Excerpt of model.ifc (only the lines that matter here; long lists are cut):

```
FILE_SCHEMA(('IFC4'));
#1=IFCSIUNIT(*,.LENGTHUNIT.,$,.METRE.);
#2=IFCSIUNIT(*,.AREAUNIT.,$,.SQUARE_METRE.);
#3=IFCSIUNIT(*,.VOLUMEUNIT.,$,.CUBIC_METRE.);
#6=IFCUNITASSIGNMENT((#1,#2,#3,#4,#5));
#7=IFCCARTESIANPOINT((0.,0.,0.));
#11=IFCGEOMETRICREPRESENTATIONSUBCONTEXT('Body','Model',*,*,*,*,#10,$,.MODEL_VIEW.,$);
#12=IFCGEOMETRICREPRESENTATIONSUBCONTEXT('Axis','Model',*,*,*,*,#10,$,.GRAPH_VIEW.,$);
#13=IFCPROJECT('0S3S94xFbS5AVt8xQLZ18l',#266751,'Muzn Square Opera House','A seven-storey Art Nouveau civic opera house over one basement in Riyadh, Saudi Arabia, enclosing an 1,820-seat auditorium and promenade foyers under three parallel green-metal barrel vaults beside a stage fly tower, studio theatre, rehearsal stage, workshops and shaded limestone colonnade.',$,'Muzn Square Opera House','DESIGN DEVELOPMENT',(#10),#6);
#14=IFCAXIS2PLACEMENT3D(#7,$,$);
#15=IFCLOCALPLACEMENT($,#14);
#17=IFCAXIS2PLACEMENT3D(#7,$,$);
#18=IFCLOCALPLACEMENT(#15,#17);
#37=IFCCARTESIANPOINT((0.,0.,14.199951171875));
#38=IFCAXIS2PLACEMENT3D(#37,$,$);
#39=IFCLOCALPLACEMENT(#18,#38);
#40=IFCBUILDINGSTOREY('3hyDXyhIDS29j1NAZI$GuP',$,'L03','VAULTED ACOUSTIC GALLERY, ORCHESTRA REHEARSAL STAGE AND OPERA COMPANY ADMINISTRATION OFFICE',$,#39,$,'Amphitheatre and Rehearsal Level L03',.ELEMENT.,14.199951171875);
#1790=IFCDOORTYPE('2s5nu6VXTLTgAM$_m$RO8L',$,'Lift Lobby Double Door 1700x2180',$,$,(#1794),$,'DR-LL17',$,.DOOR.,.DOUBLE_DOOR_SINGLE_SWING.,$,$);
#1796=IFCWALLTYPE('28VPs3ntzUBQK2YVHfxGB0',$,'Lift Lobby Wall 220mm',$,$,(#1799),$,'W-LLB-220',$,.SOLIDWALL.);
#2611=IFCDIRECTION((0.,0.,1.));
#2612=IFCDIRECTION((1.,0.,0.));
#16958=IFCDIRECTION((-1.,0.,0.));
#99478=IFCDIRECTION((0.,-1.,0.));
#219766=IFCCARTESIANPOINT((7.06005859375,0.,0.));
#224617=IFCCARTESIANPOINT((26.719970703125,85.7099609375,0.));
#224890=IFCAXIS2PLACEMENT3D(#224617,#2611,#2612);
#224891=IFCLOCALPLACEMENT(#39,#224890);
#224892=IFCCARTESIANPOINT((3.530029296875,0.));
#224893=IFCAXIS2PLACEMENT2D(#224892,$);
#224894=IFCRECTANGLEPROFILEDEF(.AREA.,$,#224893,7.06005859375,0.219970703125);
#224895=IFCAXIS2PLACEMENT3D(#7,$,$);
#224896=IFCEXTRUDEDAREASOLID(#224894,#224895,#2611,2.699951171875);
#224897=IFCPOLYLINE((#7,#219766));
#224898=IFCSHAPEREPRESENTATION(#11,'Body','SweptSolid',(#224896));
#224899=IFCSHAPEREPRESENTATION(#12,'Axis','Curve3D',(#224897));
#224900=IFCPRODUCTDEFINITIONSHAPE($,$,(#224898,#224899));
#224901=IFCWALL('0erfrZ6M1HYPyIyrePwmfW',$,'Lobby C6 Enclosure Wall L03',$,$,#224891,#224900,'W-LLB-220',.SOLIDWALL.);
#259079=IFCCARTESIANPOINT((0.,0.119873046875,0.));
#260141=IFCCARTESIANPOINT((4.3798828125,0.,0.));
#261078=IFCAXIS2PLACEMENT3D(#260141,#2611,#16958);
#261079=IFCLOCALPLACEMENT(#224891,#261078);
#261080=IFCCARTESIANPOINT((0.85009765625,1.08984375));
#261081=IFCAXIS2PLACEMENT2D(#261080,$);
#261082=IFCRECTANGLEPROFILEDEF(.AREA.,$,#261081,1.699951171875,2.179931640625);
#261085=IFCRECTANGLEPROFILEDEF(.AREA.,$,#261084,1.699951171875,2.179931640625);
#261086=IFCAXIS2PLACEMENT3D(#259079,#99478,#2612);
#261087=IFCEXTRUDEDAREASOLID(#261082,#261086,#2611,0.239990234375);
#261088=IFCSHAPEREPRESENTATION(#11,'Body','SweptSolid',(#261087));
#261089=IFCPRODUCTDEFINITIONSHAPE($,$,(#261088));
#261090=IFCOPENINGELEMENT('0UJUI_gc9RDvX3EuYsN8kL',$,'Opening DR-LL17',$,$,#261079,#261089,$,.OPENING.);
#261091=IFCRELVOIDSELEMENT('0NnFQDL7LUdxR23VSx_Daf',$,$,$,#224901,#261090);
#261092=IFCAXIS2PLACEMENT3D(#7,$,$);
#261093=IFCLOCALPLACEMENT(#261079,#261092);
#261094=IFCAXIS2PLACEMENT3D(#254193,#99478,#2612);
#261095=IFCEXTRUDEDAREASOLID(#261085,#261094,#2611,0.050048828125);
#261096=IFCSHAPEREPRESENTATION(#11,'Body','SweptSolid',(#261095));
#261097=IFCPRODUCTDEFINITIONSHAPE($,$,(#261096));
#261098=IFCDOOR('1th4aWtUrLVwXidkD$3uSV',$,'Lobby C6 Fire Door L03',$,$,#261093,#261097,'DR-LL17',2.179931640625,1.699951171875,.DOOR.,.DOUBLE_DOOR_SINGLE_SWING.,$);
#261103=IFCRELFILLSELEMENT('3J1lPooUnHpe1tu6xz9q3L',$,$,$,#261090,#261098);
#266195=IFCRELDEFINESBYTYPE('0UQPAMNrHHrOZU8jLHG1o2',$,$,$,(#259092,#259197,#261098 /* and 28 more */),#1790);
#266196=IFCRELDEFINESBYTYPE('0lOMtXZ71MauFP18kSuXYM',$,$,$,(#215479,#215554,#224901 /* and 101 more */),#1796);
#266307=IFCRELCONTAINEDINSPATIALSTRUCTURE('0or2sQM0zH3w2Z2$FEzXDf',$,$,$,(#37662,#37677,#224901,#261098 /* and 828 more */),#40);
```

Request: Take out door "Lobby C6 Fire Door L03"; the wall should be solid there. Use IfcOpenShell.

```python
import ifcopenshell
import ifcopenshell.api.feature
import ifcopenshell.api.root
import ifcopenshell.geom
import ifcopenshell.util.shape

model = ifcopenshell.open("model.ifc")
settings = ifcopenshell.geom.settings()


def volume(element):
    """Net volume in cubic metres, openings subtracted."""
    shape = ifcopenshell.geom.create_shape(settings, element)
    return ifcopenshell.util.shape.get_volume(shape.geometry)


door = model.by_guid("1th4aWtUrLVwXidkD$3uSV")
opening = door.FillsVoids[0].RelatingOpeningElement
wall = opening.VoidsElements[0].RelatingBuildingElement
before = volume(wall)

ifcopenshell.api.root.remove_product(model, product=door)
ifcopenshell.api.feature.remove_feature(model, feature=opening)

after = volume(wall)

print(f"wall volume {before:.3f} -> {after:.3f} m3")

model.write("model-out.ifc")
```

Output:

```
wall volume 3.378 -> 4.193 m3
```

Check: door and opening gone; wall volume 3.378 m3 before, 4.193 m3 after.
